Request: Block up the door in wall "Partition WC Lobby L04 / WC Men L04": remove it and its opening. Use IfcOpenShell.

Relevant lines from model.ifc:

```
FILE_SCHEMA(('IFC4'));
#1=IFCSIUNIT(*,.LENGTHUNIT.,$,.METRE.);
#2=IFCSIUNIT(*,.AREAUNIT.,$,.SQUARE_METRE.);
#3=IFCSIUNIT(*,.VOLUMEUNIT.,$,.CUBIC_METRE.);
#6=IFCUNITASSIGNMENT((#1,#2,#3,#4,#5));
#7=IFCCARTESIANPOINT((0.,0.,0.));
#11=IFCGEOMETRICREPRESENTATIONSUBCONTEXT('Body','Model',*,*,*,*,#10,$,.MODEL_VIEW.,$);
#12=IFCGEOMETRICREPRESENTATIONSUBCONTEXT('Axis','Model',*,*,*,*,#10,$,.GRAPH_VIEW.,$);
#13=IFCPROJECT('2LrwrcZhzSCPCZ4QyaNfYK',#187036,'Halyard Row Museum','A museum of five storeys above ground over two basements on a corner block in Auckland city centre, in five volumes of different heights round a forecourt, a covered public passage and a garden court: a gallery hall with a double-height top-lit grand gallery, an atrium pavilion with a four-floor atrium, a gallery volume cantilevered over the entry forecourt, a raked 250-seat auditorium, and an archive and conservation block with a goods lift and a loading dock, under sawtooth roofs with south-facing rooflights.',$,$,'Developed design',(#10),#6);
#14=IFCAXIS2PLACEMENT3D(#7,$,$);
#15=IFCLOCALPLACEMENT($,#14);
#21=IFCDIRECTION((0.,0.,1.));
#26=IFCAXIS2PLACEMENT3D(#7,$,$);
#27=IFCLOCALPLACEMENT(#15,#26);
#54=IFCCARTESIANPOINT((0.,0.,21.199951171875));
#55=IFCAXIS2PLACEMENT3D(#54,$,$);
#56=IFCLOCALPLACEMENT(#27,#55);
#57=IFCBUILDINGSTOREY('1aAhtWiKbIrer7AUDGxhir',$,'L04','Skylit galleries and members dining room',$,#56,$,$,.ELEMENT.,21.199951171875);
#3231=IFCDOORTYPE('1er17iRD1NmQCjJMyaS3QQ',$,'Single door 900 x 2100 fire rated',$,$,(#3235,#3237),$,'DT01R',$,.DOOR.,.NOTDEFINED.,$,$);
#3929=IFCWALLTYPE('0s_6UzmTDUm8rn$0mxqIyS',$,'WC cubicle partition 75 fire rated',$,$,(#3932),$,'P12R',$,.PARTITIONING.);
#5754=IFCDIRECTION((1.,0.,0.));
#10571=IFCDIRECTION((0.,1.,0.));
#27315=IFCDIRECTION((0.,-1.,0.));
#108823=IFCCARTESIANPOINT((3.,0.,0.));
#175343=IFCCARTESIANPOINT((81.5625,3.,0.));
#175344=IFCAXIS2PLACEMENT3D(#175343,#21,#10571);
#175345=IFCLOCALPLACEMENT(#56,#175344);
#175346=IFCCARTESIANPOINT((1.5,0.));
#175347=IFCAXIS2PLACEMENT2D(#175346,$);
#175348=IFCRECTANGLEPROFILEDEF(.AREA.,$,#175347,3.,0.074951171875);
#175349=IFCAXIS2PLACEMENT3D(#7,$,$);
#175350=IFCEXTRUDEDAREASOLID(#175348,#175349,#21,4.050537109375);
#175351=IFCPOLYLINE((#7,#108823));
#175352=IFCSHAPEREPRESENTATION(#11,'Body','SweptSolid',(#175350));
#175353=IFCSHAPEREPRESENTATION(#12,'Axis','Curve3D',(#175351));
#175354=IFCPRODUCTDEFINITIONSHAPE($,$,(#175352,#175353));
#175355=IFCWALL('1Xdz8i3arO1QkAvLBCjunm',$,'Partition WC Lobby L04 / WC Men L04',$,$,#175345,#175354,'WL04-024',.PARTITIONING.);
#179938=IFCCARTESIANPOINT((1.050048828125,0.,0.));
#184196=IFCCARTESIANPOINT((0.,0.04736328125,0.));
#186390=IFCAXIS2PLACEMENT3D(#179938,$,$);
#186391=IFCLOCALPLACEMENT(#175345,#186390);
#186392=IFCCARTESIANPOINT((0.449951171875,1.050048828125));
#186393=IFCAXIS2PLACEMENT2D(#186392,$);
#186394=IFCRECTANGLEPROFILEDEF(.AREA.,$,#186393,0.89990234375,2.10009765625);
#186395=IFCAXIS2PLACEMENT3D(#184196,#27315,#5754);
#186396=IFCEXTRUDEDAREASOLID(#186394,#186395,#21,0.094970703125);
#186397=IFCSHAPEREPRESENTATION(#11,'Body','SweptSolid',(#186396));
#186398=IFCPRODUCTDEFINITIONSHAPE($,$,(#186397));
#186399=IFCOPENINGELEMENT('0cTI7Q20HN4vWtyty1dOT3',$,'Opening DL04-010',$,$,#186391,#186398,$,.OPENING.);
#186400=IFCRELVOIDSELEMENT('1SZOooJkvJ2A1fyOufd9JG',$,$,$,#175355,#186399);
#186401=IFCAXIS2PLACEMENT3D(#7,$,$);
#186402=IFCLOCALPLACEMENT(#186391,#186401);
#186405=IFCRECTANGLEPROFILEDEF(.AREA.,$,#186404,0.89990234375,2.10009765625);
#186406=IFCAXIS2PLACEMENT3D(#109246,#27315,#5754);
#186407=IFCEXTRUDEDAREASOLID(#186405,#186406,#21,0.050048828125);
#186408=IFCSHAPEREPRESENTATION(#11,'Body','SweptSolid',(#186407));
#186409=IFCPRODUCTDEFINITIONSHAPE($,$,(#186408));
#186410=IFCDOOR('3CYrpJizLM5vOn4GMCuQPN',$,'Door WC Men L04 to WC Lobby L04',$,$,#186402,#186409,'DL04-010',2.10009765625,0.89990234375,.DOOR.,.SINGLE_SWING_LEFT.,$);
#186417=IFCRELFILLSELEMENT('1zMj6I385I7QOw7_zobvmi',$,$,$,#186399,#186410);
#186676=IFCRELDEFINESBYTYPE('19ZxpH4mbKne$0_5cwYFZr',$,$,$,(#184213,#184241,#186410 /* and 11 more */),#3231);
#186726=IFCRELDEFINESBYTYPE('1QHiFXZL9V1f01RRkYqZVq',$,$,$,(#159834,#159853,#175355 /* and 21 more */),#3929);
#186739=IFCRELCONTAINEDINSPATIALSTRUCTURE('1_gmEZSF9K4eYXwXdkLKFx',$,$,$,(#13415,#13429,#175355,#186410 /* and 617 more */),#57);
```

```python
import ifcopenshell
import ifcopenshell.api.feature
import ifcopenshell.api.root
import ifcopenshell.geom
import ifcopenshell.util.shape

model = ifcopenshell.open("model.ifc")
settings = ifcopenshell.geom.settings()


def volume(element):
    """Net volume in cubic metres, openings subtracted."""
    shape = ifcopenshell.geom.create_shape(settings, element)
    return ifcopenshell.util.shape.get_volume(shape.geometry)


door = model.by_id(186410)
opening = door.FillsVoids[0].RelatingOpeningElement
wall = opening.VoidsElements[0].RelatingBuildingElement
before = volume(wall)

ifcopenshell.api.root.remove_product(model, product=door)
ifcopenshell.api.feature.remove_feature(model, feature=opening)

after = volume(wall)

print(f"wall volume {before:.3f} -> {after:.3f} m3")

model.write("model_v2.ifc")
```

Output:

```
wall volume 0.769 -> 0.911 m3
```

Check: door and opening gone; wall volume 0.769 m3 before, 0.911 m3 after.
